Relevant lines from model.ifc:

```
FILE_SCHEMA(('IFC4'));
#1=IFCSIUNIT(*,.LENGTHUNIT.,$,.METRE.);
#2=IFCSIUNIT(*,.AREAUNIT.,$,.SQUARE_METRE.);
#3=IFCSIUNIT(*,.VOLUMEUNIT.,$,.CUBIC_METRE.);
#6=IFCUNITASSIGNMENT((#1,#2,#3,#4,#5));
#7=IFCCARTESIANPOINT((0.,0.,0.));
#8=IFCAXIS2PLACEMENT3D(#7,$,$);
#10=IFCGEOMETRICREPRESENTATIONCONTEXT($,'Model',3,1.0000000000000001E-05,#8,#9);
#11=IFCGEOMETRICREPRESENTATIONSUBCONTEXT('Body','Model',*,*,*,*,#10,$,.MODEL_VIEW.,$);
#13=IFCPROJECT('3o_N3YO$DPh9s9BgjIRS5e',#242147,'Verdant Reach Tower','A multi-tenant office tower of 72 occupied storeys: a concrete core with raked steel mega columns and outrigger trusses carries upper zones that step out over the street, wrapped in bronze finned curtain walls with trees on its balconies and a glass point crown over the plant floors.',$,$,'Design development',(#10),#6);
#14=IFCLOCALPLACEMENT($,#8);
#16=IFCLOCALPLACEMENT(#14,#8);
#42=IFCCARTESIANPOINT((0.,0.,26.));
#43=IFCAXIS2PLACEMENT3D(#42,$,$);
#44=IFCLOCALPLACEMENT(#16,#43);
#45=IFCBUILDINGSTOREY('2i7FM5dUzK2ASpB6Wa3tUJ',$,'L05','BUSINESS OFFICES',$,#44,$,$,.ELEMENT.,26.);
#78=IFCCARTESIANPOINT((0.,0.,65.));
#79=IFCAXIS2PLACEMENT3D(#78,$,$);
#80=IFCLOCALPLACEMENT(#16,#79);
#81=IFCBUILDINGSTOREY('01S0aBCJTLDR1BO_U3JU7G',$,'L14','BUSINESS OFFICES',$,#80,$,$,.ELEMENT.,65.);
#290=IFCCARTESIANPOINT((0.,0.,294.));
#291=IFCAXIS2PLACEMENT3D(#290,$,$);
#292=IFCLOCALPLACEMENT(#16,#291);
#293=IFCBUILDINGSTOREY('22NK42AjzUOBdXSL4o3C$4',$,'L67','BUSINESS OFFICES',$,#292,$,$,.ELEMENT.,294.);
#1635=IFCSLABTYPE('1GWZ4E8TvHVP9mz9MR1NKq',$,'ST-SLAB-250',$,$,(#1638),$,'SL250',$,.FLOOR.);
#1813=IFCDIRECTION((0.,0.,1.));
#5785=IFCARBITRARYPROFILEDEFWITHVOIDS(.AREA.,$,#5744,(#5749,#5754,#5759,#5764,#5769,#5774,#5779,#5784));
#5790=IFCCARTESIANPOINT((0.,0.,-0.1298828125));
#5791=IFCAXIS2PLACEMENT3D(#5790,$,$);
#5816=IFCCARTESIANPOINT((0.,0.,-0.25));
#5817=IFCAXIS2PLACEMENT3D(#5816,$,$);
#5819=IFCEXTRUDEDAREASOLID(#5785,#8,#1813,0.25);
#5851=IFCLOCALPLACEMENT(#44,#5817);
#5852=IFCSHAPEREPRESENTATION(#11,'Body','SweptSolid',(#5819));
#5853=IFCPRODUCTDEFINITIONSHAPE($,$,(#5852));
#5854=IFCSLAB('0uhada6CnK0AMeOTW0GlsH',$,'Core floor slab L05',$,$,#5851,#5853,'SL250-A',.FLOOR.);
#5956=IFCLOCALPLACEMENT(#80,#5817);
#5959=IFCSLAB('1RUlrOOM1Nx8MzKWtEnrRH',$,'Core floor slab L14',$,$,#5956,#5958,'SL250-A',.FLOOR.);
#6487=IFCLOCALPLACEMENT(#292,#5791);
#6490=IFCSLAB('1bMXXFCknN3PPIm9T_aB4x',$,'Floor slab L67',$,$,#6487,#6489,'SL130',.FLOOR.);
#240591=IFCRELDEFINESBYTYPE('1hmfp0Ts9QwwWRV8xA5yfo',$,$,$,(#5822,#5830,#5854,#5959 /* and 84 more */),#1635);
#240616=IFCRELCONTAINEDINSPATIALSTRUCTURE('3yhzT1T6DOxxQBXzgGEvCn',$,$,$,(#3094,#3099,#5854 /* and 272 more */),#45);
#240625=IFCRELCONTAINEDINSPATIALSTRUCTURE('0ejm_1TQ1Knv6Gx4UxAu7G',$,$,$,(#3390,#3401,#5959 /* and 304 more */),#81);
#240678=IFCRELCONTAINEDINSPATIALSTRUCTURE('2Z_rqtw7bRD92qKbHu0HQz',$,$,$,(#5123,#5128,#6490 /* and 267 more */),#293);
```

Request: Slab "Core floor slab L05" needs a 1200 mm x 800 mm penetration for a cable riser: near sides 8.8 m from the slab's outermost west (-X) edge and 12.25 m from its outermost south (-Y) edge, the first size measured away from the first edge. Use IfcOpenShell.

```python
import numpy as np
import ifcopenshell
import ifcopenshell.api.feature
import ifcopenshell.api.geometry
import ifcopenshell.api.root
import ifcopenshell.geom
import ifcopenshell.util.placement
import ifcopenshell.util.representation
import ifcopenshell.util.shape
import ifcopenshell.util.unit

model = ifcopenshell.open("model.ifc")
unit_scale = ifcopenshell.util.unit.calculate_unit_scale(model)
settings = ifcopenshell.geom.settings()


def volume(element):
    """Net volume in cubic metres, openings subtracted."""
    shape = ifcopenshell.geom.create_shape(settings, element)
    return ifcopenshell.util.shape.get_volume(shape.geometry)


slab = model.by_id(5854)
before = volume(slab)

# Extent in the slab's own axes, in metres. The edges named are its -X and -Y sides.
slab_shape = ifcopenshell.geom.create_shape(settings, slab)
vertices = ifcopenshell.util.shape.get_vertices(slab_shape.geometry)
x_min, y_min, bottom = vertices.min(axis=0)
top = vertices[:, 2].max()

opening = ifcopenshell.api.root.create_entity(model, ifc_class="IfcOpeningElement", name="Cable riser opening", predefined_type="OPENING")
context = ifcopenshell.util.representation.get_context(model, "Model", "Body", "MODEL_VIEW")
width, depth = 1.2, 0.8
outline = [(0.0, 0.0), (width, 0.0), (width, depth), (0.0, depth), (0.0, 0.0)]
# Overshoot both faces by 50 mm so the cut is clean.
shape = ifcopenshell.api.geometry.add_slab_representation(
    model, context=context, depth=top - bottom + 0.1, polyline=outline
)
ifcopenshell.api.geometry.assign_representation(model, product=opening, representation=shape)

matrix = ifcopenshell.util.placement.get_local_placement(slab.ObjectPlacement)
matrix[:, 3] = matrix @ np.append(np.array([x_min + 8.8, y_min + 12.25, bottom - 0.05]) / unit_scale, 1.0)
ifcopenshell.api.geometry.edit_object_placement(model, product=opening, matrix=matrix, is_si=False)
ifcopenshell.api.feature.add_feature(model, feature=opening, element=slab)

after = volume(slab)

print(f"slab volume {before:.3f} -> {after:.3f} m3")

model.write("model_updated.ifc")
```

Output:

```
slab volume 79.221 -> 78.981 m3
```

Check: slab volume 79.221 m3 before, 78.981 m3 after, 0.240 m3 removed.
